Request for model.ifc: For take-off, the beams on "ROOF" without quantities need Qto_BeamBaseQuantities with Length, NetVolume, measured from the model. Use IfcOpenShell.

First a look at what the model holds.

```python
import ifcopenshell
import ifcopenshell.util.element
import ifcopenshell.util.unit

model = ifcopenshell.open("model.ifc")
print(model.schema)
for unit_type in ("LENGTHUNIT", "AREAUNIT", "VOLUMEUNIT"):
    print(unit_type, ifcopenshell.util.unit.calculate_unit_scale(model, unit_type))
storey = next(s for s in model.by_type("IfcBuildingStorey") if s.Name == "ROOF")
beams = [e for e in ifcopenshell.util.element.get_decomposition(storey) if e.is_a("IfcBeam")]
for e in sorted(beams, key=lambda e: e.id()):
    print(e.id(), e.is_a(), e.Name, list(ifcopenshell.util.element.get_psets(e, qtos_only=True)), sep=" | ")
```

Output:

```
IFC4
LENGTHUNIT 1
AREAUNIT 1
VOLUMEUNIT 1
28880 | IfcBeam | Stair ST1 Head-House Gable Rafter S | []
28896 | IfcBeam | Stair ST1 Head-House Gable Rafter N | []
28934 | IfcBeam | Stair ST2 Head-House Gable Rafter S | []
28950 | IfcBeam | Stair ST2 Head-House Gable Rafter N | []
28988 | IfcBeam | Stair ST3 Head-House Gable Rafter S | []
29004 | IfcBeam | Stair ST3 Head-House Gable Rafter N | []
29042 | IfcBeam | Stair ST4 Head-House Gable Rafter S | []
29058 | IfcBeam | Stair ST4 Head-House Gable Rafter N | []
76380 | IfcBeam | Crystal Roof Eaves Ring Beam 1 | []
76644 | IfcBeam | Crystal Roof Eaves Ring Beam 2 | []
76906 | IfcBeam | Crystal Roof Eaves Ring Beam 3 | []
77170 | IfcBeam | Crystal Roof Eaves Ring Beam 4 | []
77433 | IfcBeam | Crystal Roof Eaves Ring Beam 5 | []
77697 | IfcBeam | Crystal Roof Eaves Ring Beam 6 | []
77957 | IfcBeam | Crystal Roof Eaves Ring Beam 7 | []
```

```python
import ifcopenshell
import ifcopenshell.api.pset
import ifcopenshell.geom
import ifcopenshell.util.element
import ifcopenshell.util.shape
import ifcopenshell.util.unit

model = ifcopenshell.open("model.ifc")
unit_scale = ifcopenshell.util.unit.calculate_unit_scale(model)
volume_scale = ifcopenshell.util.unit.calculate_unit_scale(model, "VOLUMEUNIT")
settings = ifcopenshell.geom.settings()

storey = next(s for s in model.by_type("IfcBuildingStorey") if s.Name == "ROOF")
beams = [e for e in ifcopenshell.util.element.get_decomposition(storey) if e.is_a("IfcBeam")]

for e in sorted(beams, key=lambda e: e.id()):
    if ifcopenshell.util.element.get_psets(e, qtos_only=True, should_inherit=False):
        continue
    # Geometry comes back in metres, in the element's own axes.
    shape = ifcopenshell.geom.create_shape(settings, e)
    values = {
        "Length": ifcopenshell.util.shape.get_max_xyz(shape.geometry) / unit_scale,
        "NetVolume": ifcopenshell.util.shape.get_volume(shape.geometry) / volume_scale,
    }
    qto = ifcopenshell.api.pset.add_qto(model, product=e, name="Qto_BeamBaseQuantities")
    ifcopenshell.api.pset.edit_qto(model, qto=qto, properties=values)
    print(e.id(), {k: round(v, 3) for k, v in values.items()})

model.write("model_v2.ifc")
```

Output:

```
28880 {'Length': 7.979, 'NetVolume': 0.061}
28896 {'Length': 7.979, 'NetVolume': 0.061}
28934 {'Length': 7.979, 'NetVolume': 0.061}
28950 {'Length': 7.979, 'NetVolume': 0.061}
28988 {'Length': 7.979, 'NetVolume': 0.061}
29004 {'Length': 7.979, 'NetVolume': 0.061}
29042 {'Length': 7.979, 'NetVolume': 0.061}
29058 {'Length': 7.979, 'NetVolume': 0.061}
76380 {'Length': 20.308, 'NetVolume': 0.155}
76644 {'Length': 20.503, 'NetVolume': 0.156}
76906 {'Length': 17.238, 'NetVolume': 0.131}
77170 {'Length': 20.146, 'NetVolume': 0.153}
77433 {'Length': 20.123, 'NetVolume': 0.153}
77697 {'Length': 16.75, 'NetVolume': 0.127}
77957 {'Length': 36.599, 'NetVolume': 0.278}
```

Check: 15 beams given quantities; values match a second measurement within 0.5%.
